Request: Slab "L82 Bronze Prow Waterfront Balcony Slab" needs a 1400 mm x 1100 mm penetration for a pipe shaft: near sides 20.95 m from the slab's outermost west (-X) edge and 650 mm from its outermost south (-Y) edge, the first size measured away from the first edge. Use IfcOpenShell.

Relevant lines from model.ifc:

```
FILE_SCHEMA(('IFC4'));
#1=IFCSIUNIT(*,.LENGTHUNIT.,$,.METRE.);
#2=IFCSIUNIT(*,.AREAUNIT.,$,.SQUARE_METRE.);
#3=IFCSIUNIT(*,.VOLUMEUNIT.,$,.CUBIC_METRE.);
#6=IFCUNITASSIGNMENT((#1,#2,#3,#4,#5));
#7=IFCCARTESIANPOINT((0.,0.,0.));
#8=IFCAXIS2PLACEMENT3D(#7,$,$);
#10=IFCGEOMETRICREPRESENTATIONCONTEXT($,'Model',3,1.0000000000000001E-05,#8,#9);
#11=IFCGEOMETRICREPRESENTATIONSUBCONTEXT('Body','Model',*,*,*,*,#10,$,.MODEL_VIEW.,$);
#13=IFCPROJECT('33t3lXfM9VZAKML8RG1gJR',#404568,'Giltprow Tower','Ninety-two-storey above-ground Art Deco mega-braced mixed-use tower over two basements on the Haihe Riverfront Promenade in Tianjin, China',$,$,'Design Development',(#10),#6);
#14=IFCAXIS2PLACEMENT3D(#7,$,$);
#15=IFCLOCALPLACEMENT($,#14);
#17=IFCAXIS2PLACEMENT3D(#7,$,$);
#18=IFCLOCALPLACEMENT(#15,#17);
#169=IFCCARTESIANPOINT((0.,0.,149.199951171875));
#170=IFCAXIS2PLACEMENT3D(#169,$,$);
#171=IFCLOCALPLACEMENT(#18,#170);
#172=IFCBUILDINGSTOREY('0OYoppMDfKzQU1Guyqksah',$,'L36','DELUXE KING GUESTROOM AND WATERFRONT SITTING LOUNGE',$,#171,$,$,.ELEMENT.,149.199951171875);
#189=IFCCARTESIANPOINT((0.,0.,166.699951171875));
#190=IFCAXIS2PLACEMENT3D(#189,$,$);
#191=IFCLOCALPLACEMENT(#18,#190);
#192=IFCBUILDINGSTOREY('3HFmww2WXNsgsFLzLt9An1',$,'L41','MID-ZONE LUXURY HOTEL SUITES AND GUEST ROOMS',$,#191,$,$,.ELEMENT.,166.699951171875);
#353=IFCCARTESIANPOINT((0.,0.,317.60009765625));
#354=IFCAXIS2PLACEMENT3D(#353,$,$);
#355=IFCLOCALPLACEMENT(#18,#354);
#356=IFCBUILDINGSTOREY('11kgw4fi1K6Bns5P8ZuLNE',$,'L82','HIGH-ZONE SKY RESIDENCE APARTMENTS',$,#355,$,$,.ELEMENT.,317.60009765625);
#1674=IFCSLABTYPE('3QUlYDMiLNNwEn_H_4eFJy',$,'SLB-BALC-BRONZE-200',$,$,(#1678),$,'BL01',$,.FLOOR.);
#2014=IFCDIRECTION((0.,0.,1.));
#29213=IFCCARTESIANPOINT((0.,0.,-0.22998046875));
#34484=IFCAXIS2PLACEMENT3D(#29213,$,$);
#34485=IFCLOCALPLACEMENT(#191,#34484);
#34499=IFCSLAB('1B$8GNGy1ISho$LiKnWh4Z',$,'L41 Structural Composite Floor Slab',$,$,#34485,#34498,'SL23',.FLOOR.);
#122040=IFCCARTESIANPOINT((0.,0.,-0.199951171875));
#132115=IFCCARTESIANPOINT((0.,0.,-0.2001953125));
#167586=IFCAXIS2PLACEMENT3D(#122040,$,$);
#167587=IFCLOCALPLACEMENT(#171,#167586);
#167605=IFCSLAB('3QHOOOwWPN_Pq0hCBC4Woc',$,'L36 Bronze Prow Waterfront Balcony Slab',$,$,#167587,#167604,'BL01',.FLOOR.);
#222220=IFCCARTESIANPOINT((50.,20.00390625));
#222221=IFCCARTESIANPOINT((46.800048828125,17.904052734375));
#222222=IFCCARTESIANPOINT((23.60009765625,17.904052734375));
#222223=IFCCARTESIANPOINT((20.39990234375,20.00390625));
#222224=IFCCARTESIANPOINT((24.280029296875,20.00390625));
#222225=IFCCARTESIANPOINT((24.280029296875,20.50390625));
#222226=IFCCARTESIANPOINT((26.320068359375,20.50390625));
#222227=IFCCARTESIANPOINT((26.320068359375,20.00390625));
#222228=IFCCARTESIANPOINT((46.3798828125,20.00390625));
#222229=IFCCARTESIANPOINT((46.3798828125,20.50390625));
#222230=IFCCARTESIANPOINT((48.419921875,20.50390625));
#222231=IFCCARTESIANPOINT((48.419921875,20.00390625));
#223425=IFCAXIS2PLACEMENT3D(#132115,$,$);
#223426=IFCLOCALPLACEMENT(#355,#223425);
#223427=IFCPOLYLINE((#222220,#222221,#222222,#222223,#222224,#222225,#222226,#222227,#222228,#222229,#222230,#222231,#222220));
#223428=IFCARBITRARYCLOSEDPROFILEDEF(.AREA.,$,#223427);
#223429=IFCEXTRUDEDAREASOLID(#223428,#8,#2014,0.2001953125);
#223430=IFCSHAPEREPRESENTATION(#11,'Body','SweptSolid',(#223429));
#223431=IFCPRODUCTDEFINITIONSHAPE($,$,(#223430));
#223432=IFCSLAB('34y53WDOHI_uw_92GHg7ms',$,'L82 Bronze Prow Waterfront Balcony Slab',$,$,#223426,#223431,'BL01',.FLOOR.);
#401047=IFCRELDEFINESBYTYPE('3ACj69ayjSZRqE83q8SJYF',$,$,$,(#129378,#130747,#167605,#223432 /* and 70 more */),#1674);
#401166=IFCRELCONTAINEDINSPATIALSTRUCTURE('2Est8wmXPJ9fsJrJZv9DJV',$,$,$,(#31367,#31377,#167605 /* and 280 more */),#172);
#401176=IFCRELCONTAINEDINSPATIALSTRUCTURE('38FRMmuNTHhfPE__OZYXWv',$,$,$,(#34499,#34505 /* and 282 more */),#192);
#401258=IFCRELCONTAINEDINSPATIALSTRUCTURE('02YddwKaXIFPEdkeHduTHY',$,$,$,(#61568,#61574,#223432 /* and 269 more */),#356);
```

```python
import numpy as np
import ifcopenshell
import ifcopenshell.api.feature
import ifcopenshell.api.geometry
import ifcopenshell.api.root
import ifcopenshell.geom
import ifcopenshell.util.placement
import ifcopenshell.util.representation
import ifcopenshell.util.shape
import ifcopenshell.util.unit

model = ifcopenshell.open("model.ifc")
unit_scale = ifcopenshell.util.unit.calculate_unit_scale(model)
settings = ifcopenshell.geom.settings()


def volume(element):
    """Net volume in cubic metres, openings subtracted."""
    shape = ifcopenshell.geom.create_shape(settings, element)
    return ifcopenshell.util.shape.get_volume(shape.geometry)


slab = model.by_guid("34y53WDOHI_uw_92GHg7ms")
before = volume(slab)

# Extent in the slab's own axes, in metres. The edges named are its -X and -Y sides.
slab_shape = ifcopenshell.geom.create_shape(settings, slab)
vertices = ifcopenshell.util.shape.get_vertices(slab_shape.geometry)
x_min, y_min, bottom = vertices.min(axis=0)
top = vertices[:, 2].max()

opening = ifcopenshell.api.root.create_entity(model, ifc_class="IfcOpeningElement", name="Pipe shaft opening", predefined_type="OPENING")
context = ifcopenshell.util.representation.get_context(model, "Model", "Body", "MODEL_VIEW")
width, depth = 1.4, 1.1
outline = [(0.0, 0.0), (width, 0.0), (width, depth), (0.0, depth), (0.0, 0.0)]
# Overshoot both faces by 50 mm so the cut is clean.
shape = ifcopenshell.api.geometry.add_slab_representation(
    model, context=context, depth=top - bottom + 0.1, polyline=outline
)
ifcopenshell.api.geometry.assign_representation(model, product=opening, representation=shape)

matrix = ifcopenshell.util.placement.get_local_placement(slab.ObjectPlacement)
matrix[:, 3] = matrix @ np.append(np.array([x_min + 20.95, y_min + 0.65, bottom - 0.05]) / unit_scale, 1.0)
ifcopenshell.api.geometry.edit_object_placement(model, product=opening, matrix=matrix, is_si=False)
ifcopenshell.api.feature.add_feature(model, feature=opening, element=slab)

after = volume(slab)

print(f"slab volume {before:.3f} -> {after:.3f} m3")

model.write("model_rev.ifc")
```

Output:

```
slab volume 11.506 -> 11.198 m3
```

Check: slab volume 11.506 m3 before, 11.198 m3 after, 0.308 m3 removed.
